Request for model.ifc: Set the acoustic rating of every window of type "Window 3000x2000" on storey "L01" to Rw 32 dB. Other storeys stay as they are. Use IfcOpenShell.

First a look at what the model holds.

```python
import ifcopenshell
import ifcopenshell.util.element

model = ifcopenshell.open("model.ifc")
print(model.schema)
storey = next(s for s in model.by_type("IfcBuildingStorey") if s.Name == "L01")
windows = [e for e in ifcopenshell.util.element.get_decomposition(storey) if e.is_a("IfcWindow")]
seen = {}
for e in windows:
    element_type = ifcopenshell.util.element.get_type(e)
    key = (element_type.Name if element_type != e and element_type else None, ifcopenshell.util.element.get_pset(e, "Pset_WindowCommon", "AcousticRating"))
    seen[key] = seen.get(key, 0) + 1
for (name, value), count in sorted(seen.items(), key=str):
    print(count, "x", name, "|", value)
```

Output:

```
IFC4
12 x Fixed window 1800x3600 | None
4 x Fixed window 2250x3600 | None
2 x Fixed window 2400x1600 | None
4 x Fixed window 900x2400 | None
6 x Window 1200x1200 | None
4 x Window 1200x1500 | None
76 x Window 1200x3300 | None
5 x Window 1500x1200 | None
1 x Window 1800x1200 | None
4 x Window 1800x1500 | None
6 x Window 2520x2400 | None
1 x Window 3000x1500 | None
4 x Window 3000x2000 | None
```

```python
import ifcopenshell
import ifcopenshell.api.pset
import ifcopenshell.util.element

model = ifcopenshell.open("model.ifc")

storey = next(s for s in model.by_type("IfcBuildingStorey") if s.Name == "L01")
windows = [e for e in ifcopenshell.util.element.get_decomposition(storey) if e.is_a("IfcWindow")]

count = 0
for e in windows:
    element_type = ifcopenshell.util.element.get_type(e)
    if element_type in (None, e) or element_type.Name != "Window 3000x2000":
        continue
    # add_pset returns the element's existing set when there is one.
    pset = ifcopenshell.api.pset.add_pset(model, product=e, name="Pset_WindowCommon")
    ifcopenshell.api.pset.edit_pset(model, pset=pset, properties={"AcousticRating": "Rw 32 dB"})
    count += 1

print(count, "windows updated")

model.write("model_edited.ifc")
```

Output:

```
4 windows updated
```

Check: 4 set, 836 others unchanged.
